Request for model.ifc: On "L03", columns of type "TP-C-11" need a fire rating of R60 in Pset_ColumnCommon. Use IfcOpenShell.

First a look at what the model holds.

```python
import ifcopenshell
import ifcopenshell.util.element

model = ifcopenshell.open("model.ifc")
print(model.schema)
storey = next(s for s in model.by_type("IfcBuildingStorey") if s.Name == "L03")
columns = [e for e in ifcopenshell.util.element.get_decomposition(storey) if e.is_a("IfcColumn")]
seen = {}
for e in columns:
    element_type = ifcopenshell.util.element.get_type(e)
    key = (element_type.Name if element_type != e and element_type else None, ifcopenshell.util.element.get_pset(e, "Pset_ColumnCommon", "FireRating"))
    seen[key] = seen.get(key, 0) + 1
for (name, value), count in sorted(seen.items(), key=str):
    print(count, "x", name, "|", value)
```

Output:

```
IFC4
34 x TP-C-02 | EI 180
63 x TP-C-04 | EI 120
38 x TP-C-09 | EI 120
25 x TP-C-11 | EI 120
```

```python
import ifcopenshell
import ifcopenshell.api.pset
import ifcopenshell.util.element

model = ifcopenshell.open("model.ifc")

storey = next(s for s in model.by_type("IfcBuildingStorey") if s.Name == "L03")
columns = [e for e in ifcopenshell.util.element.get_decomposition(storey) if e.is_a("IfcColumn")]

count = 0
for e in columns:
    element_type = ifcopenshell.util.element.get_type(e)
    if element_type in (None, e) or element_type.Name != "TP-C-11":
        continue
    # add_pset returns the element's existing set when there is one.
    pset = ifcopenshell.api.pset.add_pset(model, product=e, name="Pset_ColumnCommon")
    ifcopenshell.api.pset.edit_pset(model, pset=pset, properties={"FireRating": "R60"})
    count += 1

print(count, "columns updated")

model.write("model_updated.ifc")
```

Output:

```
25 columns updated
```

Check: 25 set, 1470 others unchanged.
